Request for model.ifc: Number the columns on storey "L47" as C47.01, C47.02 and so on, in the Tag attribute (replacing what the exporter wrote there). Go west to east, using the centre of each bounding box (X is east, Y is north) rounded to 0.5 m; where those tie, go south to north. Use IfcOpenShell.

First a look at what the model holds.

```python
import ifcopenshell
import ifcopenshell.util.element
import ifcopenshell.util.placement

model = ifcopenshell.open("model.ifc")
print(model.schema)
storey = next(s for s in model.by_type("IfcBuildingStorey") if s.Name == "L47")
columns = [e for e in ifcopenshell.util.element.get_decomposition(storey) if e.is_a("IfcColumn")]
for e in sorted(columns, key=lambda e: e.id()):
    origin = ifcopenshell.util.placement.get_local_placement(e.ObjectPlacement)[:3, 3]
    print(e.id(), e.Tag, e.Name, origin.round(2) + 0.0, sep=" | ")
```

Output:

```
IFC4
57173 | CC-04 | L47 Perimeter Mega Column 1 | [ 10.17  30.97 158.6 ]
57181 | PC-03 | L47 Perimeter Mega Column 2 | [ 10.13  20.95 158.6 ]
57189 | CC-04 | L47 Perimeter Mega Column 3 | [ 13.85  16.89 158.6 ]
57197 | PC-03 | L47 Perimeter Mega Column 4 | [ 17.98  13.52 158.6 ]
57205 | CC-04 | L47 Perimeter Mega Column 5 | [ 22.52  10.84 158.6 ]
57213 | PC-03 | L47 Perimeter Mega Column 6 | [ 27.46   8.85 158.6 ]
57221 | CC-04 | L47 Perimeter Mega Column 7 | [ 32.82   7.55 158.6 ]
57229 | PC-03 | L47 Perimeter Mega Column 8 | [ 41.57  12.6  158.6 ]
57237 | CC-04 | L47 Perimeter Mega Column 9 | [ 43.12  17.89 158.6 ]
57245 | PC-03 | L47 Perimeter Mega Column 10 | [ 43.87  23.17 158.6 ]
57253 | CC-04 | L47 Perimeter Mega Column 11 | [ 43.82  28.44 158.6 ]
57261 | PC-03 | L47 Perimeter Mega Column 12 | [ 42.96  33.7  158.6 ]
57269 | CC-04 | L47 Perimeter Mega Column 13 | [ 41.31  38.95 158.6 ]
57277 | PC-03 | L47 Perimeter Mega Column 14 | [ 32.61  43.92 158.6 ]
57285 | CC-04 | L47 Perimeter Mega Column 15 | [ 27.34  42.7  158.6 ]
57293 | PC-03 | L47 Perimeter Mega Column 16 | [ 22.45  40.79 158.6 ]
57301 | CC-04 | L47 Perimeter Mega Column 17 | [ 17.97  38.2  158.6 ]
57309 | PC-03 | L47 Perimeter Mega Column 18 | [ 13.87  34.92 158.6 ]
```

```python
import ifcopenshell
import ifcopenshell.geom
import ifcopenshell.util.element
import ifcopenshell.util.shape

model = ifcopenshell.open("model.ifc")
settings = ifcopenshell.geom.settings()
settings.set("use-world-coords", True)


def centre(element):
    shape = ifcopenshell.geom.create_shape(settings, element)
    return ifcopenshell.util.shape.get_bbox_centroid(shape.geometry)


storey = next(s for s in model.by_type("IfcBuildingStorey") if s.Name == "L47")
columns = [e for e in ifcopenshell.util.element.get_decomposition(storey) if e.is_a("IfcColumn")]

# Insertion points can sit at a corner or the storey origin, so sort by the geometry (in metres).
centres = {e: centre(e) for e in columns}
columns.sort(key=lambda e: (round(centres[e][0] / 0.5), centres[e][1]))

for i, e in enumerate(columns, start=1):
    number = f"C47.{i:02d}"
    e.Tag = number
    print(e.id(), number)

model.write("model_rev.ifc")
```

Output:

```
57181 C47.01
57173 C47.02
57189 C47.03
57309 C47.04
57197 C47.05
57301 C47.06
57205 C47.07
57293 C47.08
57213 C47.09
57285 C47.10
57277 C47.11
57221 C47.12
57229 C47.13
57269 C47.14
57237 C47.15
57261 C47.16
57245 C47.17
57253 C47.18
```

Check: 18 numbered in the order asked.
